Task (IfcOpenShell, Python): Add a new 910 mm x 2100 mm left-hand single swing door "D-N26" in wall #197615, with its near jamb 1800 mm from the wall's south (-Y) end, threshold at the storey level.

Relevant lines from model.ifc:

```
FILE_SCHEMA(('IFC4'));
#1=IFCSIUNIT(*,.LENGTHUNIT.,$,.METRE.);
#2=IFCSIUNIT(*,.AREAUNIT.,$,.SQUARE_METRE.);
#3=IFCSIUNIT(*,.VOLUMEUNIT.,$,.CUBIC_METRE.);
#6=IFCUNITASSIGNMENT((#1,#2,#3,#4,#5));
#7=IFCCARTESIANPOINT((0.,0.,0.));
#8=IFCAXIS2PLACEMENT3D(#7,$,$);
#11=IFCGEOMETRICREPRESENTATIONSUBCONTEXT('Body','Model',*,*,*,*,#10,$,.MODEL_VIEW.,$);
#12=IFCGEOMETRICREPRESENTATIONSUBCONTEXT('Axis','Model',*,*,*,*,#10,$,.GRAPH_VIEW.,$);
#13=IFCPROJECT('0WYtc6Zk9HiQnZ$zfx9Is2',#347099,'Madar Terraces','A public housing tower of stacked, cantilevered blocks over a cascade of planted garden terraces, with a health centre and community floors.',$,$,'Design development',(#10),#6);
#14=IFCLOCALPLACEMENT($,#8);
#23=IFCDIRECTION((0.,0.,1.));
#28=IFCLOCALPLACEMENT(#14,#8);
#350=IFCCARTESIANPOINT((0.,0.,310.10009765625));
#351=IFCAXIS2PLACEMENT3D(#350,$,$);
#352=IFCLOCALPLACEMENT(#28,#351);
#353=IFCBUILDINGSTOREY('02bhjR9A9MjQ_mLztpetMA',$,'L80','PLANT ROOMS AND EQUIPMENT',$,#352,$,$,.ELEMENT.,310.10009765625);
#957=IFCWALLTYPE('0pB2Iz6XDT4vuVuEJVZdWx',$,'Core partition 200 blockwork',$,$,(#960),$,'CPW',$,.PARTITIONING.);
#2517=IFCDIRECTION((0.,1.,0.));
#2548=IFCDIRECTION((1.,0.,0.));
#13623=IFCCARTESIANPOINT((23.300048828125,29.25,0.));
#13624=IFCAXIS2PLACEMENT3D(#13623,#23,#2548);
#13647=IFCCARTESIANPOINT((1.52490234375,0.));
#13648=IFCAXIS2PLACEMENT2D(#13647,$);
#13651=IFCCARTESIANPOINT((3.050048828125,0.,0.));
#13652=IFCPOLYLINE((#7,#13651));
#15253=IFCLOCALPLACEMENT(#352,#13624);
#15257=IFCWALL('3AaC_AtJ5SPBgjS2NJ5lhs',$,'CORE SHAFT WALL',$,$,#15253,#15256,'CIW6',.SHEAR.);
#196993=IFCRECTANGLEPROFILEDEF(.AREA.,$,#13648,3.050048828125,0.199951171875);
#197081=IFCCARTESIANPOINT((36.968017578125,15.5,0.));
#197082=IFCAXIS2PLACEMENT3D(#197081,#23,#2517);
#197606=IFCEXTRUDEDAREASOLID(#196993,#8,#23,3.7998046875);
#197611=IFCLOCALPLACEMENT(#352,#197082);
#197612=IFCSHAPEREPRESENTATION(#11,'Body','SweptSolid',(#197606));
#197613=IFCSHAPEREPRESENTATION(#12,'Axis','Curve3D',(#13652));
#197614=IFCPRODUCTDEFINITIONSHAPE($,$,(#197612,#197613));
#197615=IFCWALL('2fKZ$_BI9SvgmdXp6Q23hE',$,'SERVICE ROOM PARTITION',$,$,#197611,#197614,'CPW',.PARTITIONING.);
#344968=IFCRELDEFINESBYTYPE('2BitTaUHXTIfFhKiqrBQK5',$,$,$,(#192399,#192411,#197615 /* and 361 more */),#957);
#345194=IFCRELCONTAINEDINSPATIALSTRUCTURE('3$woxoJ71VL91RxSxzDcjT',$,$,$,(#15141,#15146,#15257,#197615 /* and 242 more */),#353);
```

```python
import numpy as np
import ifcopenshell
import ifcopenshell.api.feature
import ifcopenshell.api.geometry
import ifcopenshell.api.root
import ifcopenshell.api.spatial
import ifcopenshell.geom
import ifcopenshell.util.element
import ifcopenshell.util.placement
import ifcopenshell.util.representation
import ifcopenshell.util.shape
import ifcopenshell.util.unit

model = ifcopenshell.open("model.ifc")
unit_scale = ifcopenshell.util.unit.calculate_unit_scale(model)
settings = ifcopenshell.geom.settings()


def volume(element):
    """Net volume in cubic metres, openings subtracted."""
    shape = ifcopenshell.geom.create_shape(settings, element)
    return ifcopenshell.util.shape.get_volume(shape.geometry)


wall = model.by_guid("2fKZ$_BI9SvgmdXp6Q23hE")
storey = ifcopenshell.util.element.get_container(wall, ifc_class="IfcBuildingStorey")
context = ifcopenshell.util.representation.get_context(model, "Model", "Body", "MODEL_VIEW")
before = volume(wall)

width, height, from_end, sill = 0.91, 2.1, 1.8, 0.0  # metres

# The wall runs along its own X axis, and the end named is its -X end.
wall_shape = ifcopenshell.geom.create_shape(settings, wall)
x, y, z = ifcopenshell.util.shape.get_vertices(wall_shape.geometry).T
start = x.min() + from_end
face, thickness = float(y.min()), float(y.max() - y.min())
wall_matrix = ifcopenshell.util.placement.get_local_placement(wall.ObjectPlacement)
level = ifcopenshell.util.placement.get_local_placement(storey.ObjectPlacement)[2, 3]


def in_wall(x, y):
    """Placement at x, y metres in the wall's axes, at sill height."""
    matrix = wall_matrix.copy()
    matrix[:, 3] = wall_matrix @ np.array([x / unit_scale, y / unit_scale, 0.0, 1.0])
    matrix[2, 3] = level + sill / unit_scale
    return matrix


# Opening: a box that overshoots both wall faces by 50 mm.
opening = ifcopenshell.api.root.create_entity(model, ifc_class="IfcOpeningElement", predefined_type="OPENING")
box = ifcopenshell.api.geometry.add_wall_representation(
    model, context=context, length=width, height=height, thickness=thickness + 0.1
)
ifcopenshell.api.geometry.assign_representation(model, product=opening, representation=box)
ifcopenshell.api.geometry.edit_object_placement(model, product=opening, matrix=in_wall(start, face - 0.05), is_si=False)
ifcopenshell.api.feature.add_feature(model, feature=opening, element=wall)

door = ifcopenshell.api.root.create_entity(model, ifc_class="IfcDoor", name="D-N26", predefined_type="DOOR")
door.OverallWidth, door.OverallHeight = width / unit_scale, height / unit_scale
door.OperationType = "SINGLE_SWING_LEFT"
body = ifcopenshell.api.geometry.add_door_representation(
    model,
    context=context,
    overall_width=door.OverallWidth,
    overall_height=door.OverallHeight,
    operation_type="SINGLE_SWING_LEFT",
    lining_properties={"LiningDepth": thickness / unit_scale, "ThresholdDepth": thickness / unit_scale},
)
ifcopenshell.api.geometry.assign_representation(model, product=door, representation=body)
ifcopenshell.api.spatial.assign_container(model, products=[door], relating_structure=storey)
ifcopenshell.api.feature.add_filling(model, opening=opening, element=door)

# The lining spans the wall, so the door starts at the wall face.
ifcopenshell.api.geometry.edit_object_placement(model, product=door, matrix=in_wall(start, face), is_si=False)

after = volume(wall)

print(f"wall volume {before:.3f} -> {after:.3f} m3")

model.write("model-out.ifc")
```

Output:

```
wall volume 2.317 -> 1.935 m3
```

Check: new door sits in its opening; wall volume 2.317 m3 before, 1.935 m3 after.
